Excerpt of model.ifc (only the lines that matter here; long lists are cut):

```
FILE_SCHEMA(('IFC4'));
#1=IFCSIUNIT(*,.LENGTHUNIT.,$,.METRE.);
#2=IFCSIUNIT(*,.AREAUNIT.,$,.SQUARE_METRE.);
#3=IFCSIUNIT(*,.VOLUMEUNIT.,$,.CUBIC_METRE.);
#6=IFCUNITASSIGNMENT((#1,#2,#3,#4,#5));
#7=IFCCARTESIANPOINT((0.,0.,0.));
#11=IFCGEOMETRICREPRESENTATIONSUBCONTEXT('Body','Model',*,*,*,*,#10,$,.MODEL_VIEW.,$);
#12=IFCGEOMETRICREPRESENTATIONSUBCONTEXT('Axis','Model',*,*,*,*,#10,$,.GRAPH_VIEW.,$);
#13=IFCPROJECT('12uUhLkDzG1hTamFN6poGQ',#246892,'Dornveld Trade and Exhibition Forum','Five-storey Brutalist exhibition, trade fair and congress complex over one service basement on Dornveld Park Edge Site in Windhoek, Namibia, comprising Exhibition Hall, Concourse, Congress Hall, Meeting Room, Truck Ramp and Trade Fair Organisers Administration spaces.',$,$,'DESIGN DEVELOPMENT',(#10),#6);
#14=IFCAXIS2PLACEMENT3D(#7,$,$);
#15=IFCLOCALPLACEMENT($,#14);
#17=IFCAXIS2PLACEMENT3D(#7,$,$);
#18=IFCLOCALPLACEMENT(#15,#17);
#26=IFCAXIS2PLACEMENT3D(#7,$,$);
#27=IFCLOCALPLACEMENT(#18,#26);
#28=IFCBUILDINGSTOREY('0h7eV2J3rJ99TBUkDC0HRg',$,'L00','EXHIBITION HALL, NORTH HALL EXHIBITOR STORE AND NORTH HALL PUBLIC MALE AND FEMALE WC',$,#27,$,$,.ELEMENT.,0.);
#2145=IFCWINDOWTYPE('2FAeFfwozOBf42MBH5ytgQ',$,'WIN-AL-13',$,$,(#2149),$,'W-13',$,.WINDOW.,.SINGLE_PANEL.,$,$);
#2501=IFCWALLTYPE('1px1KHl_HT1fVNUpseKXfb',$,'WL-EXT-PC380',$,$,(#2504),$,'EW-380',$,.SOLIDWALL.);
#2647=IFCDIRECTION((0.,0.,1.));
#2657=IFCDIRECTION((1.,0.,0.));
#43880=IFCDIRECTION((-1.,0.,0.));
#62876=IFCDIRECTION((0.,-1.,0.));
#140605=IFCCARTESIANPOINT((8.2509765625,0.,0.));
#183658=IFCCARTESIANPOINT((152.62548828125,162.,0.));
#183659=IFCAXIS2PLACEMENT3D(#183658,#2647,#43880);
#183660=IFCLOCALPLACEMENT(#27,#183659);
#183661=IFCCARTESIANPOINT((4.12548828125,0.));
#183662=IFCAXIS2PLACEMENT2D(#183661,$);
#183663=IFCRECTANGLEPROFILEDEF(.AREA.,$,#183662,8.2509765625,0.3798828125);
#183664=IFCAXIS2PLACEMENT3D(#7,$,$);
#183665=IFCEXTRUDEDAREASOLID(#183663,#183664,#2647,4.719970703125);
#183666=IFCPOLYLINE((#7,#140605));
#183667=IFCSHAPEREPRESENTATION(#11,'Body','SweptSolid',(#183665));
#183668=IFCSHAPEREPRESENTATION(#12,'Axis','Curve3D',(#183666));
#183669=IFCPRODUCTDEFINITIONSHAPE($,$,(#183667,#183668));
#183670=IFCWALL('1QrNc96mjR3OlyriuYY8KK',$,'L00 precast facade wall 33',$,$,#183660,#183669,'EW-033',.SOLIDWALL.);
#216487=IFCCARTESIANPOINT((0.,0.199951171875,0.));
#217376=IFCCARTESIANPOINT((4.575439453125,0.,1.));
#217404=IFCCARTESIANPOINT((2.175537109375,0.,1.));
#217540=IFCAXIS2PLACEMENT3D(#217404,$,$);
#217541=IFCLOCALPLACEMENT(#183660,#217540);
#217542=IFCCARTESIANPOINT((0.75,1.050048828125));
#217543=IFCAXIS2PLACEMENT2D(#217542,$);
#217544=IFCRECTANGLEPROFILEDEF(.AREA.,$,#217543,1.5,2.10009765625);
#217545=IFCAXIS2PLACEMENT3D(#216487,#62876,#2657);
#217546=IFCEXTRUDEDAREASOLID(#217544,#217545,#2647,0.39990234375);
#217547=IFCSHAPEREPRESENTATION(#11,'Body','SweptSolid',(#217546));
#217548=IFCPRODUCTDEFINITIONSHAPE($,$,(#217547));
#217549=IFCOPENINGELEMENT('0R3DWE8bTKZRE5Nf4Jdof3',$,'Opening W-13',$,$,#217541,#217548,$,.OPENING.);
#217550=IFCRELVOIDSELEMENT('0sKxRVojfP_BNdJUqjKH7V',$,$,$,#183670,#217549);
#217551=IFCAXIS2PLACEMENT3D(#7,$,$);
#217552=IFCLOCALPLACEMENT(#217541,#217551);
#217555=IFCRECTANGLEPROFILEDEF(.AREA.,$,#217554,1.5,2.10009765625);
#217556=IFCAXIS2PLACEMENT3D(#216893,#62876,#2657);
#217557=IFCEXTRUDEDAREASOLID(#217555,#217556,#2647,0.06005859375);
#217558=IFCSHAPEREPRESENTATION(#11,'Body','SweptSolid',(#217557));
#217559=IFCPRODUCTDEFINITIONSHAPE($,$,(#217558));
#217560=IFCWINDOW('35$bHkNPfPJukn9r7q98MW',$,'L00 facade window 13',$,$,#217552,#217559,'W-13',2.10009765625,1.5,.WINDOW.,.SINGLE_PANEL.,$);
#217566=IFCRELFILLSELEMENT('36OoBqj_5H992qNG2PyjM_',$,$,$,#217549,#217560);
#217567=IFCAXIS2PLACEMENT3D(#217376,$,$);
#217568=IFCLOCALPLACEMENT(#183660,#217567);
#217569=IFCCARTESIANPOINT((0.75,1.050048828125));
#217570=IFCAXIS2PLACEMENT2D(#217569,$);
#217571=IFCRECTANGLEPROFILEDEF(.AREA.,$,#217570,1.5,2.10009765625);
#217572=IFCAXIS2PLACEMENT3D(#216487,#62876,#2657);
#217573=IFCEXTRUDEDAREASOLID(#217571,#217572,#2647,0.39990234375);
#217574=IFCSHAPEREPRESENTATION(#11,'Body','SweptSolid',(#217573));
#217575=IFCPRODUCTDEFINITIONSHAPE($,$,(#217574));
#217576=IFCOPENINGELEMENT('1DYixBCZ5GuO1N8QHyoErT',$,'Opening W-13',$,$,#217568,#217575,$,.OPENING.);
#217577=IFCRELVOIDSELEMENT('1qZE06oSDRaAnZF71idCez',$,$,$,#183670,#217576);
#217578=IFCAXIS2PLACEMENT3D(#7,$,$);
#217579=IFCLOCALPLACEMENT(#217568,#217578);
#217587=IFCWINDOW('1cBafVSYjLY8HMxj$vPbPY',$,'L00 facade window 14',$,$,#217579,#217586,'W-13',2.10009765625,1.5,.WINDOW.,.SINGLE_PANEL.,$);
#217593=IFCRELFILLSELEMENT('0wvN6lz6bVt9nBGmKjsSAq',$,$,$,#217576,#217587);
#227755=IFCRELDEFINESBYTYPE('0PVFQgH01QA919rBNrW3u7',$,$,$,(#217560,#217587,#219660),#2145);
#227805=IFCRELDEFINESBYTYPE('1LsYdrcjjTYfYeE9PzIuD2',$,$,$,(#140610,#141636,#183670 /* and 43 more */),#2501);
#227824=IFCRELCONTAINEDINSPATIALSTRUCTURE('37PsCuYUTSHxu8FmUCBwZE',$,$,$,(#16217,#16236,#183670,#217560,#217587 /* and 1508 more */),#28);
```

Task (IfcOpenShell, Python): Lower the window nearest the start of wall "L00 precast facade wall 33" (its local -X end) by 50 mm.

```python
import numpy as np
import ifcopenshell
import ifcopenshell.api.geometry
import ifcopenshell.util.placement
import ifcopenshell.util.unit

model = ifcopenshell.open("model.ifc")
unit_scale = ifcopenshell.util.unit.calculate_unit_scale(model)

window = model.by_id(217560)
opening = window.FillsVoids[0].RelatingOpeningElement
dz = -0.05 / unit_scale

shift = np.array([0.0, 0.0, dz])
# The window is placed relative to its opening, so it follows when the opening moves.
matrix = ifcopenshell.util.placement.get_local_placement(opening.ObjectPlacement)
matrix[:3, 3] += shift
ifcopenshell.api.geometry.edit_object_placement(
    model, product=opening, matrix=matrix, is_si=False, should_transform_children=True
)

print(f"moved by {dz * unit_scale:+.3f} m")

model.write("model_v2.ifc")
```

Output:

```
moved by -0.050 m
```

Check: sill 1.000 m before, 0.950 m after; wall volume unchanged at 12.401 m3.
